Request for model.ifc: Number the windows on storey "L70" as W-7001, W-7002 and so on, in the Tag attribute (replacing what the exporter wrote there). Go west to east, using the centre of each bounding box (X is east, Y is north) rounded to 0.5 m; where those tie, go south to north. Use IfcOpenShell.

First a look at what the model holds.

```python
import ifcopenshell
import ifcopenshell.util.element
import ifcopenshell.util.placement

model = ifcopenshell.open("model.ifc")
print(model.schema)
storey = next(s for s in model.by_type("IfcBuildingStorey") if s.Name == "L70")
windows = [e for e in ifcopenshell.util.element.get_decomposition(storey) if e.is_a("IfcWindow")]
for e in sorted(windows, key=lambda e: e.id()):
    origin = ifcopenshell.util.placement.get_local_placement(e.ObjectPlacement)[:3, 3]
    print(e.id(), e.Tag, e.Name, origin.round(2) + 0.0, sep=" | ")
```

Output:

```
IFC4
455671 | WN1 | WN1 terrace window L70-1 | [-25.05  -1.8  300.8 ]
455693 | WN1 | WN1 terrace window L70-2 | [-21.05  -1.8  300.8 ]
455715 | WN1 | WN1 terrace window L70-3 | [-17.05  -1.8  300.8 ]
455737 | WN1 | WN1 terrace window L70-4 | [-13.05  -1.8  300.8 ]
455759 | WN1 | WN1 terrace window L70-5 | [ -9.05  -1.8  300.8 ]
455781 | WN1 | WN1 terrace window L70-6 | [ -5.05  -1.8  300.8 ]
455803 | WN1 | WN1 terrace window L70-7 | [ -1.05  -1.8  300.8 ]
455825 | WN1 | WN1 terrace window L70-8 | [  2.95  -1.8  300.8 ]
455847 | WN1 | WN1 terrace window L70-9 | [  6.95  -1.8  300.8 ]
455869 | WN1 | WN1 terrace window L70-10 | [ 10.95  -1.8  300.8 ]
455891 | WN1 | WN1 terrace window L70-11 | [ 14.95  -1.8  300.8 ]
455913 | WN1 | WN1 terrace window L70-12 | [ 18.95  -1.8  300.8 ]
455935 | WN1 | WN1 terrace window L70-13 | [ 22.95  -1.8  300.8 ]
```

```python
import ifcopenshell
import ifcopenshell.geom
import ifcopenshell.util.element
import ifcopenshell.util.shape

model = ifcopenshell.open("model.ifc")
settings = ifcopenshell.geom.settings()
settings.set("use-world-coords", True)


def centre(element):
    shape = ifcopenshell.geom.create_shape(settings, element)
    return ifcopenshell.util.shape.get_bbox_centroid(shape.geometry)


storey = next(s for s in model.by_type("IfcBuildingStorey") if s.Name == "L70")
windows = [e for e in ifcopenshell.util.element.get_decomposition(storey) if e.is_a("IfcWindow")]

# Insertion points can sit at a corner or the storey origin, so sort by the geometry (in metres).
centres = {e: centre(e) for e in windows}
windows.sort(key=lambda e: (round(centres[e][0] / 0.5), centres[e][1]))

for i, e in enumerate(windows, start=1):
    number = f"W-70{i:02d}"
    e.Tag = number
    print(e.id(), number)

model.write("model-out.ifc")
```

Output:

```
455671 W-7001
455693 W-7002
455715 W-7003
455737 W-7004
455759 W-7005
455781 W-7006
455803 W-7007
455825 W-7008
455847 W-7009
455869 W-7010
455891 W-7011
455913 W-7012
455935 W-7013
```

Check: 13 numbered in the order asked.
